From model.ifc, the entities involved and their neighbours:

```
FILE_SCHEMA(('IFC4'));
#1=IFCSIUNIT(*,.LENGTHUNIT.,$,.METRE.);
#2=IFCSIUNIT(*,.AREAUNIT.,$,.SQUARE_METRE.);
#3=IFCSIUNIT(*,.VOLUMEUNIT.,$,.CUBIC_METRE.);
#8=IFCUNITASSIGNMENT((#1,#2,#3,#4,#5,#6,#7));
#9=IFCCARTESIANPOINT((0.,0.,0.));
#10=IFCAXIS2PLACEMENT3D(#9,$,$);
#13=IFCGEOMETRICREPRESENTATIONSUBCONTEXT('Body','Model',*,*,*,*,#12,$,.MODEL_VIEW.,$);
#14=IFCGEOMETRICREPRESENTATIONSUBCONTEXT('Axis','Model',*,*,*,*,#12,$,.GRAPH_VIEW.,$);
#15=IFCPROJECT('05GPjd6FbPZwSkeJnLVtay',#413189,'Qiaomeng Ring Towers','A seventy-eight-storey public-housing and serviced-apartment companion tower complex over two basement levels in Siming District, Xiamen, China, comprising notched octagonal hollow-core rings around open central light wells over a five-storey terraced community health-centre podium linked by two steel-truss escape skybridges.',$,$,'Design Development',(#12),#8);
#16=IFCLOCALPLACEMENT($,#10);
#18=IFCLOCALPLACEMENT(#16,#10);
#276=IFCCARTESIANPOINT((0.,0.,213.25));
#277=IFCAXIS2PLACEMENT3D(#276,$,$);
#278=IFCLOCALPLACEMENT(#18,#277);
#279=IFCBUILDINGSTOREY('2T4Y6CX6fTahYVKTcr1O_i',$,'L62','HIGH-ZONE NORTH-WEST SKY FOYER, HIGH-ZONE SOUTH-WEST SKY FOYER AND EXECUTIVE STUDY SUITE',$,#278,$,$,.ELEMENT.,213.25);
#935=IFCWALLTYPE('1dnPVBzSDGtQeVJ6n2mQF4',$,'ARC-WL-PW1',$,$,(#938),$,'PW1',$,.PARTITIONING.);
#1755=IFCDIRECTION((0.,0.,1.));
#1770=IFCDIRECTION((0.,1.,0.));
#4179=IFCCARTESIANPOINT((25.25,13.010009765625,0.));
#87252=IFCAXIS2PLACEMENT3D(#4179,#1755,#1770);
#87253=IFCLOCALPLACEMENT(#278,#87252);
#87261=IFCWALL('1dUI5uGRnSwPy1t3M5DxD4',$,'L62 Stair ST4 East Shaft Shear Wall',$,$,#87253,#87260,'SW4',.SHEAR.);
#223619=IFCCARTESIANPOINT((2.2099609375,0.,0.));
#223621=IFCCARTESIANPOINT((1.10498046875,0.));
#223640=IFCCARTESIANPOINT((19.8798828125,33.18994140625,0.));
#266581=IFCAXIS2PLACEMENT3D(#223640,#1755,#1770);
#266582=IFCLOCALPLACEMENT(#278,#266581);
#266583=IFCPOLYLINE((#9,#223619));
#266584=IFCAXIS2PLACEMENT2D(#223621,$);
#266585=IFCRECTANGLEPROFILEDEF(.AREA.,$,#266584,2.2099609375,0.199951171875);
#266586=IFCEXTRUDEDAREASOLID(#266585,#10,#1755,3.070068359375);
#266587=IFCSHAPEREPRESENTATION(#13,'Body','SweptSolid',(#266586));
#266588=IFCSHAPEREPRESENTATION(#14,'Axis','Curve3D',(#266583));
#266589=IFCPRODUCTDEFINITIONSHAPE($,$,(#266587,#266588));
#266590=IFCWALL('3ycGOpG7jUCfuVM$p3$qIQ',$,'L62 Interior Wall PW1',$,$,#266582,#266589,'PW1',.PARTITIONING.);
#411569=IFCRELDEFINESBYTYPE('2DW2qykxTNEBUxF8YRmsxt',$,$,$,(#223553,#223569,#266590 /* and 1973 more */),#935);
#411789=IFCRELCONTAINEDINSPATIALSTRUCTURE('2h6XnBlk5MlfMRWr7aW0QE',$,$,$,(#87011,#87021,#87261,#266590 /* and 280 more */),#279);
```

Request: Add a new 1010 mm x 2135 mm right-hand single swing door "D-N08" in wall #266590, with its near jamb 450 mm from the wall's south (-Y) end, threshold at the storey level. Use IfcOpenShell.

```python
import numpy as np
import ifcopenshell
import ifcopenshell.api.feature
import ifcopenshell.api.geometry
import ifcopenshell.api.root
import ifcopenshell.api.spatial
import ifcopenshell.geom
import ifcopenshell.util.element
import ifcopenshell.util.placement
import ifcopenshell.util.representation
import ifcopenshell.util.shape
import ifcopenshell.util.unit

model = ifcopenshell.open("model.ifc")
unit_scale = ifcopenshell.util.unit.calculate_unit_scale(model)
settings = ifcopenshell.geom.settings()


def volume(element):
    """Net volume in cubic metres, openings subtracted."""
    shape = ifcopenshell.geom.create_shape(settings, element)
    return ifcopenshell.util.shape.get_volume(shape.geometry)


wall = model.by_guid("3ycGOpG7jUCfuVM$p3$qIQ")
storey = ifcopenshell.util.element.get_container(wall, ifc_class="IfcBuildingStorey")
context = ifcopenshell.util.representation.get_context(model, "Model", "Body", "MODEL_VIEW")
before = volume(wall)

width, height, from_end, sill = 1.01, 2.135, 0.45, 0.0  # metres

# The wall runs along its own X axis, and the end named is its -X end.
wall_shape = ifcopenshell.geom.create_shape(settings, wall)
x, y, z = ifcopenshell.util.shape.get_vertices(wall_shape.geometry).T
start = x.min() + from_end
face, thickness = float(y.min()), float(y.max() - y.min())
wall_matrix = ifcopenshell.util.placement.get_local_placement(wall.ObjectPlacement)
level = ifcopenshell.util.placement.get_local_placement(storey.ObjectPlacement)[2, 3]


def in_wall(x, y):
    """Placement at x, y metres in the wall's axes, at sill height."""
    matrix = wall_matrix.copy()
    matrix[:, 3] = wall_matrix @ np.array([x / unit_scale, y / unit_scale, 0.0, 1.0])
    matrix[2, 3] = level + sill / unit_scale
    return matrix


# Opening: a box that overshoots both wall faces by 50 mm.
opening = ifcopenshell.api.root.create_entity(model, ifc_class="IfcOpeningElement", predefined_type="OPENING")
box = ifcopenshell.api.geometry.add_wall_representation(
    model, context=context, length=width, height=height, thickness=thickness + 0.1
)
ifcopenshell.api.geometry.assign_representation(model, product=opening, representation=box)
ifcopenshell.api.geometry.edit_object_placement(model, product=opening, matrix=in_wall(start, face - 0.05), is_si=False)
ifcopenshell.api.feature.add_feature(model, feature=opening, element=wall)

door = ifcopenshell.api.root.create_entity(model, ifc_class="IfcDoor", name="D-N08", predefined_type="DOOR")
door.OverallWidth, door.OverallHeight = width / unit_scale, height / unit_scale
door.OperationType = "SINGLE_SWING_RIGHT"
body = ifcopenshell.api.geometry.add_door_representation(
    model,
    context=context,
    overall_width=door.OverallWidth,
    overall_height=door.OverallHeight,
    operation_type="SINGLE_SWING_RIGHT",
    lining_properties={"LiningDepth": thickness / unit_scale, "ThresholdDepth": thickness / unit_scale},
)
ifcopenshell.api.geometry.assign_representation(model, product=door, representation=body)
ifcopenshell.api.spatial.assign_container(model, products=[door], relating_structure=storey)
ifcopenshell.api.feature.add_filling(model, opening=opening, element=door)

# The lining spans the wall, so the door starts at the wall face.
ifcopenshell.api.geometry.edit_object_placement(model, product=door, matrix=in_wall(start, face), is_si=False)

after = volume(wall)

print(f"wall volume {before:.3f} -> {after:.3f} m3")

model.write("model_rev.ifc")
```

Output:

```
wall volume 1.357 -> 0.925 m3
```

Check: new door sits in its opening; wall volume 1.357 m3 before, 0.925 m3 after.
